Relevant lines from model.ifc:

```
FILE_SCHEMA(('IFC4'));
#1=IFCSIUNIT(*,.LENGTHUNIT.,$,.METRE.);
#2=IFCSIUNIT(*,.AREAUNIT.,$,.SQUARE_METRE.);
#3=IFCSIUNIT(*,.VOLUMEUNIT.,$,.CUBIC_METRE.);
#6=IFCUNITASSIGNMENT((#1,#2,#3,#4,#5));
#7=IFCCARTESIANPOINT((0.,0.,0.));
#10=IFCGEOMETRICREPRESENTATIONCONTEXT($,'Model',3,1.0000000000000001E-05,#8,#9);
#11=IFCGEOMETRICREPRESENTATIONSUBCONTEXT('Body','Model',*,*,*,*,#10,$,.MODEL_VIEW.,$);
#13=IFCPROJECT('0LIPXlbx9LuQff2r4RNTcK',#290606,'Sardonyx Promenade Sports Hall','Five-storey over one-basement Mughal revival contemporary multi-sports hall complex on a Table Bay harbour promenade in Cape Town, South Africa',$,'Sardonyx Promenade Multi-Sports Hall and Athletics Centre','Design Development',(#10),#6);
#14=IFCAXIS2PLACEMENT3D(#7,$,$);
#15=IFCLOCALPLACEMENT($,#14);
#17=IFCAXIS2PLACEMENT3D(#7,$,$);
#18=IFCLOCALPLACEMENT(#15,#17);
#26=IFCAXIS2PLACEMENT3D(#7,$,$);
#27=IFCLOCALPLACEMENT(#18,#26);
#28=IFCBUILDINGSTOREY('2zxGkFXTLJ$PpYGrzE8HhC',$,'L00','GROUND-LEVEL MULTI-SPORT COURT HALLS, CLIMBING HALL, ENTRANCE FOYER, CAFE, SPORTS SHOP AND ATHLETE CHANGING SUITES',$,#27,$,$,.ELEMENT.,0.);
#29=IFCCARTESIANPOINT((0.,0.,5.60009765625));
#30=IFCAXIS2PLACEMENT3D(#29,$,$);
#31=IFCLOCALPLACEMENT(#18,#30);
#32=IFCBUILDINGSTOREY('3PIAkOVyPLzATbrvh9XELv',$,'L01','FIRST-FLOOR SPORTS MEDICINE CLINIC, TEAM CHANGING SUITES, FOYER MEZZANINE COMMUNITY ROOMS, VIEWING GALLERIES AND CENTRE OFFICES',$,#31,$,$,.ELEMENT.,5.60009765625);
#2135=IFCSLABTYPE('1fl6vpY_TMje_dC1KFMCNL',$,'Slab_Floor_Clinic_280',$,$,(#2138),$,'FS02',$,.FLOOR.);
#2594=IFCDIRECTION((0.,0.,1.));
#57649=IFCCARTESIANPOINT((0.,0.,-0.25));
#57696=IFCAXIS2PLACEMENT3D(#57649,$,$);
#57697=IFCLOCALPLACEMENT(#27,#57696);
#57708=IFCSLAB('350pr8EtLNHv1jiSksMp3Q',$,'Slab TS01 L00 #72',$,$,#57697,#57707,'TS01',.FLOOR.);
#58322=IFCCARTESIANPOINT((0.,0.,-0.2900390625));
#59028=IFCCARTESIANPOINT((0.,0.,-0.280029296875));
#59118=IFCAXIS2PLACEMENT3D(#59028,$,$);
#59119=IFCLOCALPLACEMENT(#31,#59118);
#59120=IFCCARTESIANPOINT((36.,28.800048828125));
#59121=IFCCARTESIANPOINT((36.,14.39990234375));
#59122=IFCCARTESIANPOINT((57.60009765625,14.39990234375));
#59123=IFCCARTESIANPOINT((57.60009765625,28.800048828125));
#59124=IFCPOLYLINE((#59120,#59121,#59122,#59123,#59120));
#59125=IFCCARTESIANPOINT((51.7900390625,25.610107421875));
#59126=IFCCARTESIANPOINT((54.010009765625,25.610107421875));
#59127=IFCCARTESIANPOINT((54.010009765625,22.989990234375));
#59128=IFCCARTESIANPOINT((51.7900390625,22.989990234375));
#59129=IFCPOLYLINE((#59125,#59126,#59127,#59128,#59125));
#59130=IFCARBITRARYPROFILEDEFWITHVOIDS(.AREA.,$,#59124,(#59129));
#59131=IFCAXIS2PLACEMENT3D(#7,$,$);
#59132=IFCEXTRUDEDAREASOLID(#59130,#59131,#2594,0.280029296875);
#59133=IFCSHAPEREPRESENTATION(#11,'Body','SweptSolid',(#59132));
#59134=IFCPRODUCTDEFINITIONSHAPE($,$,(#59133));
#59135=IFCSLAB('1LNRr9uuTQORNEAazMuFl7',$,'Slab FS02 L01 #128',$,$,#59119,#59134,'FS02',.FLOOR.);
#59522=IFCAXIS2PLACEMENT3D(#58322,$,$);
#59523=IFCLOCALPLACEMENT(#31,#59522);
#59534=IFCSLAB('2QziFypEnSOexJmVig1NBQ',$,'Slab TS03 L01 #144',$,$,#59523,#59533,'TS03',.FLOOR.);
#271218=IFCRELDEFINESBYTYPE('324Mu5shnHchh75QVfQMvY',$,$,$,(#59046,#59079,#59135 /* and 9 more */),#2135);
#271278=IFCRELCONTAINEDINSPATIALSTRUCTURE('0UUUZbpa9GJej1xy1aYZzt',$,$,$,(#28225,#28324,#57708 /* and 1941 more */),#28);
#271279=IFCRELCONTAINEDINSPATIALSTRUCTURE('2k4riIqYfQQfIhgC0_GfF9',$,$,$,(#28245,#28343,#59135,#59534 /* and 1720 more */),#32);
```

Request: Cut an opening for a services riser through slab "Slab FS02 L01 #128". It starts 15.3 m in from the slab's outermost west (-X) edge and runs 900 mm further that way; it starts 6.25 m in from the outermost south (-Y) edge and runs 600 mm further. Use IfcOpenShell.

```python
import numpy as np
import ifcopenshell
import ifcopenshell.api.feature
import ifcopenshell.api.geometry
import ifcopenshell.api.root
import ifcopenshell.geom
import ifcopenshell.util.placement
import ifcopenshell.util.representation
import ifcopenshell.util.shape
import ifcopenshell.util.unit

model = ifcopenshell.open("model.ifc")
unit_scale = ifcopenshell.util.unit.calculate_unit_scale(model)
settings = ifcopenshell.geom.settings()


def volume(element):
    """Net volume in cubic metres, openings subtracted."""
    shape = ifcopenshell.geom.create_shape(settings, element)
    return ifcopenshell.util.shape.get_volume(shape.geometry)


slab = model.by_guid("1LNRr9uuTQORNEAazMuFl7")
before = volume(slab)

# Extent in the slab's own axes, in metres. The edges named are its -X and -Y sides.
slab_shape = ifcopenshell.geom.create_shape(settings, slab)
vertices = ifcopenshell.util.shape.get_vertices(slab_shape.geometry)
x_min, y_min, bottom = vertices.min(axis=0)
top = vertices[:, 2].max()

opening = ifcopenshell.api.root.create_entity(model, ifc_class="IfcOpeningElement", name="Services riser opening", predefined_type="OPENING")
context = ifcopenshell.util.representation.get_context(model, "Model", "Body", "MODEL_VIEW")
width, depth = 0.9, 0.6
outline = [(0.0, 0.0), (width, 0.0), (width, depth), (0.0, depth), (0.0, 0.0)]
# Overshoot both faces by 50 mm so the cut is clean.
shape = ifcopenshell.api.geometry.add_slab_representation(
    model, context=context, depth=top - bottom + 0.1, polyline=outline
)
ifcopenshell.api.geometry.assign_representation(model, product=opening, representation=shape)

matrix = ifcopenshell.util.placement.get_local_placement(slab.ObjectPlacement)
matrix[:, 3] = matrix @ np.append(np.array([x_min + 15.3, y_min + 6.25, bottom - 0.05]) / unit_scale, 1.0)
ifcopenshell.api.geometry.edit_object_placement(model, product=opening, matrix=matrix, is_si=False)
ifcopenshell.api.feature.add_feature(model, feature=opening, element=slab)

after = volume(slab)

print(f"slab volume {before:.3f} -> {after:.3f} m3")

model.write("model_updated.ifc")
```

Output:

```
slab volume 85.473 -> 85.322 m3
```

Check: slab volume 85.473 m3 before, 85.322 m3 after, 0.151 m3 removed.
